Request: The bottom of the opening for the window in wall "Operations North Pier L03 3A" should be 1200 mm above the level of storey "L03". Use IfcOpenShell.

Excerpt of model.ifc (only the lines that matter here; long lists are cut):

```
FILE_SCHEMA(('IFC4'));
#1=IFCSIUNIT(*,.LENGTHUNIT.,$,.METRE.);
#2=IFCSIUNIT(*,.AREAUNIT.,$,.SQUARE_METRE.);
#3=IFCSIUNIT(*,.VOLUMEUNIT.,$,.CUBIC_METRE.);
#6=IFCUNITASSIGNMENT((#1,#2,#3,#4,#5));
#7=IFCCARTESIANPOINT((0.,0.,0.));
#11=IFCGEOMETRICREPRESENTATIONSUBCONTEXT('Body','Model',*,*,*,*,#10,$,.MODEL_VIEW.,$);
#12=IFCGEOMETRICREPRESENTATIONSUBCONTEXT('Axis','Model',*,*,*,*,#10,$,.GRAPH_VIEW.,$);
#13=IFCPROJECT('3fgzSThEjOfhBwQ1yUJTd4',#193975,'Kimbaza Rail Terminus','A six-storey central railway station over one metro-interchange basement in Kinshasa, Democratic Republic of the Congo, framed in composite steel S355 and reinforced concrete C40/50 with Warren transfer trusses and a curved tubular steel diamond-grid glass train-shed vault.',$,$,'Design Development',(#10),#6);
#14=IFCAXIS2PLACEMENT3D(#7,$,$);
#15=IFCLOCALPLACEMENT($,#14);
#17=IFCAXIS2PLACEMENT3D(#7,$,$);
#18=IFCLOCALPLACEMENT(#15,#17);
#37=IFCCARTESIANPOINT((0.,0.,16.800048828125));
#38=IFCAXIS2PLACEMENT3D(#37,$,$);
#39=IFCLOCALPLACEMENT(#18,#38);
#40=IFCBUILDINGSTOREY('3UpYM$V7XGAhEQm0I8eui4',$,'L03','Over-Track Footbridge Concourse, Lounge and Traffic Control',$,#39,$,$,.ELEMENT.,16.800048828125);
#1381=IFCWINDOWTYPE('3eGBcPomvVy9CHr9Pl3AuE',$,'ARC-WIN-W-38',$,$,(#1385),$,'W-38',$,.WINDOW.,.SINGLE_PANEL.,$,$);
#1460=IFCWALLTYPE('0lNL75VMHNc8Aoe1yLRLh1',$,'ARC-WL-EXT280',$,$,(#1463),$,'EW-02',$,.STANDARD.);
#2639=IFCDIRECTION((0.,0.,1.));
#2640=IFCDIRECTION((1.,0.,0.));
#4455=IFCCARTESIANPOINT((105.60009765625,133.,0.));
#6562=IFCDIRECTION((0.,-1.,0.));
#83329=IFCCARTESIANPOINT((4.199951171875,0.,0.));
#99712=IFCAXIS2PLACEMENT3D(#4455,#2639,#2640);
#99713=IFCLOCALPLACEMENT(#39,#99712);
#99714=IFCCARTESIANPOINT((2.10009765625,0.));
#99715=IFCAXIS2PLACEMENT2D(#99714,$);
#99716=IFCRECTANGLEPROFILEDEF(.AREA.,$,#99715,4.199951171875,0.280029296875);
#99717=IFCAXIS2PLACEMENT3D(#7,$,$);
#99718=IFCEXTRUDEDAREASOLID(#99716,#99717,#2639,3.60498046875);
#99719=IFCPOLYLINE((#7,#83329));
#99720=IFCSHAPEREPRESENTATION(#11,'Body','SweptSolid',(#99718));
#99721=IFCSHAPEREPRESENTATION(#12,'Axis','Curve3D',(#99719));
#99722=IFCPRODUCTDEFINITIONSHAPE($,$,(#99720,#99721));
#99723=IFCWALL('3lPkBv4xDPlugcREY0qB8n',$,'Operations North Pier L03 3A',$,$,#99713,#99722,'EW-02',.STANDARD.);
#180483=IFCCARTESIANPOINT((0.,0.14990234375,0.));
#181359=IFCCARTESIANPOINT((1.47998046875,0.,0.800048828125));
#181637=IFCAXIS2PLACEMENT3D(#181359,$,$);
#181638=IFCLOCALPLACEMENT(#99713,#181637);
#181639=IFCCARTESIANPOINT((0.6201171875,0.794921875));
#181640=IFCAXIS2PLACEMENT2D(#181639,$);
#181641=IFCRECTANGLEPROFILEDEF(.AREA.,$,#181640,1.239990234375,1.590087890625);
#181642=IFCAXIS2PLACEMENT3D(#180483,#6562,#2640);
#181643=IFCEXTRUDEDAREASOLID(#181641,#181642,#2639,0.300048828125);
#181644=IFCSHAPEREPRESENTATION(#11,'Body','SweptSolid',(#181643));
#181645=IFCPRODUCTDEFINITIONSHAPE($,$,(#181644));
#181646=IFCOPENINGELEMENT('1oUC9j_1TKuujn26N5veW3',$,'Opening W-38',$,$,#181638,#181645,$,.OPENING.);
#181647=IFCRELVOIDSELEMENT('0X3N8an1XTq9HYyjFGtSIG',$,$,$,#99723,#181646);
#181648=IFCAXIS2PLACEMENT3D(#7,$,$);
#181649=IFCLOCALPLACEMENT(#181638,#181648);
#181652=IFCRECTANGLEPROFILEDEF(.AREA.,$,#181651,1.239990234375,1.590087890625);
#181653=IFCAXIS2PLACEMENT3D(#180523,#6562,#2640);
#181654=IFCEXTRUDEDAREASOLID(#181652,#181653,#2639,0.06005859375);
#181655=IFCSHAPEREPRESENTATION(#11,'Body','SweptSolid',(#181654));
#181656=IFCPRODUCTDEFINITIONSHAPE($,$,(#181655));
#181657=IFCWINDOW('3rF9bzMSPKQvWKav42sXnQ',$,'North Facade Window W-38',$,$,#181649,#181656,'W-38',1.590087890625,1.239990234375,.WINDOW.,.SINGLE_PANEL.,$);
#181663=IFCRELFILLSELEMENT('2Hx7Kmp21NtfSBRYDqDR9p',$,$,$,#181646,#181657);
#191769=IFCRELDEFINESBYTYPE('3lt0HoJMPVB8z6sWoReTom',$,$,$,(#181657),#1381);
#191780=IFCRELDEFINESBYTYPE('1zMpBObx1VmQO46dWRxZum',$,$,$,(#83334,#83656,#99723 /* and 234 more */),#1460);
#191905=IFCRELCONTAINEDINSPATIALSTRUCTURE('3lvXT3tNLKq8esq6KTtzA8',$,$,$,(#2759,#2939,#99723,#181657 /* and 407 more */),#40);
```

```python
import numpy as np
import ifcopenshell
import ifcopenshell.api.geometry
import ifcopenshell.geom
import ifcopenshell.util.element
import ifcopenshell.util.placement
import ifcopenshell.util.shape
import ifcopenshell.util.unit

model = ifcopenshell.open("model.ifc")
unit_scale = ifcopenshell.util.unit.calculate_unit_scale(model)

window = model.by_guid("3rF9bzMSPKQvWKav42sXnQ")
opening = window.FillsVoids[0].RelatingOpeningElement
storey = ifcopenshell.util.element.get_container(window, ifc_class="IfcBuildingStorey")
level = ifcopenshell.util.placement.get_local_placement(storey.ObjectPlacement)[2, 3]

# The opening's origin need not be at the sill, so measure its lowest point.
shape = ifcopenshell.geom.create_shape(ifcopenshell.geom.settings(), opening)
bottom = ifcopenshell.util.shape.get_shape_bottom_elevation(shape, shape.geometry) / unit_scale
dz = level + 1.2 / unit_scale - bottom

shift = np.array([0.0, 0.0, dz])
# The window is placed relative to its opening, so it follows when the opening moves.
matrix = ifcopenshell.util.placement.get_local_placement(opening.ObjectPlacement)
matrix[:3, 3] += shift
ifcopenshell.api.geometry.edit_object_placement(
    model, product=opening, matrix=matrix, is_si=False, should_transform_children=True
)

print(f"moved by {dz * unit_scale:+.3f} m")

model.write("model_updated.ifc")
```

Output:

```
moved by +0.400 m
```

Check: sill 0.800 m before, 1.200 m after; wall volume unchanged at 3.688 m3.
